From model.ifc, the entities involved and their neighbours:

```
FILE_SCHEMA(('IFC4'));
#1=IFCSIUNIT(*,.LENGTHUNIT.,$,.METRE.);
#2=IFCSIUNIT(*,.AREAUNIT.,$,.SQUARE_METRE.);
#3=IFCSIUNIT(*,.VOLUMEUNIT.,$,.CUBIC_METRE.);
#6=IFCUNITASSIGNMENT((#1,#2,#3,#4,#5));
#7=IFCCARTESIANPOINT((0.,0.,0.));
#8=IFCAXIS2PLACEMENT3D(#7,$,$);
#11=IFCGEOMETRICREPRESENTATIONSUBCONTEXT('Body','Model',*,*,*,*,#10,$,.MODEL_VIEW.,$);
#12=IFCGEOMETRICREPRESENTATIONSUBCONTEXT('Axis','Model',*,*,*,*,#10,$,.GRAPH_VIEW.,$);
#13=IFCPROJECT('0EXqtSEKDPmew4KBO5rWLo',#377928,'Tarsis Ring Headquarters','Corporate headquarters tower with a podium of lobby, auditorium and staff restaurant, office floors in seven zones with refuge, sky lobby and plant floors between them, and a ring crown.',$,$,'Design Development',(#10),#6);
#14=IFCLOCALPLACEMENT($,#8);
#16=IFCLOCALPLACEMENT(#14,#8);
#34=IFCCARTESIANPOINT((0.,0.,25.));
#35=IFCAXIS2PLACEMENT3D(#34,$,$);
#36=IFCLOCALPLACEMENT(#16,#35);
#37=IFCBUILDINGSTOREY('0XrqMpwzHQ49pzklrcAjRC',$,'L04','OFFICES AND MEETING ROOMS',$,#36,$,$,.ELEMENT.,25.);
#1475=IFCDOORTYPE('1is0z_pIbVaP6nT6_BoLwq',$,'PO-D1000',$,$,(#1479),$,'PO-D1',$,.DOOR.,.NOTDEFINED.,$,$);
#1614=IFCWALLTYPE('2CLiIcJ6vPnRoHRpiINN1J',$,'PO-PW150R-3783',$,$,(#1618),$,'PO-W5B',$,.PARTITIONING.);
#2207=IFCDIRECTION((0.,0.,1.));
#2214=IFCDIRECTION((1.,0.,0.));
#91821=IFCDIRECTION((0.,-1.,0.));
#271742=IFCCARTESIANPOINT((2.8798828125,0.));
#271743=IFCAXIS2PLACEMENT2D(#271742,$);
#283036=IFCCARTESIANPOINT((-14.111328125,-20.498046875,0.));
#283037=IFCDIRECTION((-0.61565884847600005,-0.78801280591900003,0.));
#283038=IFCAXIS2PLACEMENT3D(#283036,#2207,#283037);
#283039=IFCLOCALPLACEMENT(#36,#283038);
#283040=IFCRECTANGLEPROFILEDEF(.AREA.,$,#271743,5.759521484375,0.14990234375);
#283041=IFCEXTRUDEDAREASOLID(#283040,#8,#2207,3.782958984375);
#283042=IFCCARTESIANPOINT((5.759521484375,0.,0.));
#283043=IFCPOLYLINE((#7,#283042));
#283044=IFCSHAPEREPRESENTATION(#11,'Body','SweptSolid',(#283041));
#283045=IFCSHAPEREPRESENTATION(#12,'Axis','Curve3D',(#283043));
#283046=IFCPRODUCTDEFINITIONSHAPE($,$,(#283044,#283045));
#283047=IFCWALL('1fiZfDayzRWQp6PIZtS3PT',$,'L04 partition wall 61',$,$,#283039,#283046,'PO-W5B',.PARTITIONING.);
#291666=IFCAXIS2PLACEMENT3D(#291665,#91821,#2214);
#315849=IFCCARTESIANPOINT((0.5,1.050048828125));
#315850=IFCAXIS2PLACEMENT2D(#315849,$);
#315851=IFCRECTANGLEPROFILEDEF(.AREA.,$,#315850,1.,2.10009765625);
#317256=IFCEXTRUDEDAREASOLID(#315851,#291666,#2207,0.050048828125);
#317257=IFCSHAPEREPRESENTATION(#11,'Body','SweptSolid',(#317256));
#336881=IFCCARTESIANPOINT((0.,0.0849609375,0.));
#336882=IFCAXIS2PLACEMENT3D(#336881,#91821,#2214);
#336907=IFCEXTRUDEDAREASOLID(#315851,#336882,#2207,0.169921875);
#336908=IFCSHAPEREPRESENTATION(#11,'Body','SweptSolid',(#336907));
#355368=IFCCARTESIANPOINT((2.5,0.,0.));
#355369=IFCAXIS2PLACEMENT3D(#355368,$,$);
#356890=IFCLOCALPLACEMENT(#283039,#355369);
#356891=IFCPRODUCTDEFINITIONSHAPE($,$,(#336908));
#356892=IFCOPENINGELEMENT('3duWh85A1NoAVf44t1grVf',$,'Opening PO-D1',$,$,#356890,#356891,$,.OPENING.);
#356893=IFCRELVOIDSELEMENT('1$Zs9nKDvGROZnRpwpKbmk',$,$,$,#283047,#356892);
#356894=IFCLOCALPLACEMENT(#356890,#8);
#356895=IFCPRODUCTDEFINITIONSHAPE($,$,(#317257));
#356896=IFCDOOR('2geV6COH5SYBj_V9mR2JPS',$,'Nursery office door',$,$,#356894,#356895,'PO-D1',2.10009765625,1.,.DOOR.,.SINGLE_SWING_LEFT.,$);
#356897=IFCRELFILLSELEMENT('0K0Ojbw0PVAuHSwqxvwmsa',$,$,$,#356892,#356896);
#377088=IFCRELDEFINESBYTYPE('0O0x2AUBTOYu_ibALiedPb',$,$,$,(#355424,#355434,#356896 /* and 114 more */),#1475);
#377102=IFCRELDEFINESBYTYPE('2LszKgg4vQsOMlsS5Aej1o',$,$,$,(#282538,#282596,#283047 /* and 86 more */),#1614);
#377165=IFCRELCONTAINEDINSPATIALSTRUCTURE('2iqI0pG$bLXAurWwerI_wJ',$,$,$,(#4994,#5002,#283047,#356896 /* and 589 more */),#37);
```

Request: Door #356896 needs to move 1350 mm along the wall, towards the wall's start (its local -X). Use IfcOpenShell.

```python
import ifcopenshell
import ifcopenshell.api.geometry
import ifcopenshell.util.placement

model = ifcopenshell.open("model.ifc")

door = model.by_guid("2geV6COH5SYBj_V9mR2JPS")
opening = door.FillsVoids[0].RelatingOpeningElement
wall = opening.VoidsElements[0].RelatingBuildingElement

wall_matrix = ifcopenshell.util.placement.get_local_placement(wall.ObjectPlacement)
shift = wall_matrix[:3, 0] * -1.35
before = ifcopenshell.util.placement.get_local_placement(door.ObjectPlacement)[:3, 3].copy()

# The door is placed relative to its opening, so it follows when the opening moves.
matrix = ifcopenshell.util.placement.get_local_placement(opening.ObjectPlacement)
matrix[:3, 3] += shift
ifcopenshell.api.geometry.edit_object_placement(
    model, product=opening, matrix=matrix, is_si=False, should_transform_children=True
)

after = ifcopenshell.util.placement.get_local_placement(door.ObjectPlacement)[:3, 3]
print("door moved by", (after - before).round(3) + 0.0)

model.write("model-out.ifc")
```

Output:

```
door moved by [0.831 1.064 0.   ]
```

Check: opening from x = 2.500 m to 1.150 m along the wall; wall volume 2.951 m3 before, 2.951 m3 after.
